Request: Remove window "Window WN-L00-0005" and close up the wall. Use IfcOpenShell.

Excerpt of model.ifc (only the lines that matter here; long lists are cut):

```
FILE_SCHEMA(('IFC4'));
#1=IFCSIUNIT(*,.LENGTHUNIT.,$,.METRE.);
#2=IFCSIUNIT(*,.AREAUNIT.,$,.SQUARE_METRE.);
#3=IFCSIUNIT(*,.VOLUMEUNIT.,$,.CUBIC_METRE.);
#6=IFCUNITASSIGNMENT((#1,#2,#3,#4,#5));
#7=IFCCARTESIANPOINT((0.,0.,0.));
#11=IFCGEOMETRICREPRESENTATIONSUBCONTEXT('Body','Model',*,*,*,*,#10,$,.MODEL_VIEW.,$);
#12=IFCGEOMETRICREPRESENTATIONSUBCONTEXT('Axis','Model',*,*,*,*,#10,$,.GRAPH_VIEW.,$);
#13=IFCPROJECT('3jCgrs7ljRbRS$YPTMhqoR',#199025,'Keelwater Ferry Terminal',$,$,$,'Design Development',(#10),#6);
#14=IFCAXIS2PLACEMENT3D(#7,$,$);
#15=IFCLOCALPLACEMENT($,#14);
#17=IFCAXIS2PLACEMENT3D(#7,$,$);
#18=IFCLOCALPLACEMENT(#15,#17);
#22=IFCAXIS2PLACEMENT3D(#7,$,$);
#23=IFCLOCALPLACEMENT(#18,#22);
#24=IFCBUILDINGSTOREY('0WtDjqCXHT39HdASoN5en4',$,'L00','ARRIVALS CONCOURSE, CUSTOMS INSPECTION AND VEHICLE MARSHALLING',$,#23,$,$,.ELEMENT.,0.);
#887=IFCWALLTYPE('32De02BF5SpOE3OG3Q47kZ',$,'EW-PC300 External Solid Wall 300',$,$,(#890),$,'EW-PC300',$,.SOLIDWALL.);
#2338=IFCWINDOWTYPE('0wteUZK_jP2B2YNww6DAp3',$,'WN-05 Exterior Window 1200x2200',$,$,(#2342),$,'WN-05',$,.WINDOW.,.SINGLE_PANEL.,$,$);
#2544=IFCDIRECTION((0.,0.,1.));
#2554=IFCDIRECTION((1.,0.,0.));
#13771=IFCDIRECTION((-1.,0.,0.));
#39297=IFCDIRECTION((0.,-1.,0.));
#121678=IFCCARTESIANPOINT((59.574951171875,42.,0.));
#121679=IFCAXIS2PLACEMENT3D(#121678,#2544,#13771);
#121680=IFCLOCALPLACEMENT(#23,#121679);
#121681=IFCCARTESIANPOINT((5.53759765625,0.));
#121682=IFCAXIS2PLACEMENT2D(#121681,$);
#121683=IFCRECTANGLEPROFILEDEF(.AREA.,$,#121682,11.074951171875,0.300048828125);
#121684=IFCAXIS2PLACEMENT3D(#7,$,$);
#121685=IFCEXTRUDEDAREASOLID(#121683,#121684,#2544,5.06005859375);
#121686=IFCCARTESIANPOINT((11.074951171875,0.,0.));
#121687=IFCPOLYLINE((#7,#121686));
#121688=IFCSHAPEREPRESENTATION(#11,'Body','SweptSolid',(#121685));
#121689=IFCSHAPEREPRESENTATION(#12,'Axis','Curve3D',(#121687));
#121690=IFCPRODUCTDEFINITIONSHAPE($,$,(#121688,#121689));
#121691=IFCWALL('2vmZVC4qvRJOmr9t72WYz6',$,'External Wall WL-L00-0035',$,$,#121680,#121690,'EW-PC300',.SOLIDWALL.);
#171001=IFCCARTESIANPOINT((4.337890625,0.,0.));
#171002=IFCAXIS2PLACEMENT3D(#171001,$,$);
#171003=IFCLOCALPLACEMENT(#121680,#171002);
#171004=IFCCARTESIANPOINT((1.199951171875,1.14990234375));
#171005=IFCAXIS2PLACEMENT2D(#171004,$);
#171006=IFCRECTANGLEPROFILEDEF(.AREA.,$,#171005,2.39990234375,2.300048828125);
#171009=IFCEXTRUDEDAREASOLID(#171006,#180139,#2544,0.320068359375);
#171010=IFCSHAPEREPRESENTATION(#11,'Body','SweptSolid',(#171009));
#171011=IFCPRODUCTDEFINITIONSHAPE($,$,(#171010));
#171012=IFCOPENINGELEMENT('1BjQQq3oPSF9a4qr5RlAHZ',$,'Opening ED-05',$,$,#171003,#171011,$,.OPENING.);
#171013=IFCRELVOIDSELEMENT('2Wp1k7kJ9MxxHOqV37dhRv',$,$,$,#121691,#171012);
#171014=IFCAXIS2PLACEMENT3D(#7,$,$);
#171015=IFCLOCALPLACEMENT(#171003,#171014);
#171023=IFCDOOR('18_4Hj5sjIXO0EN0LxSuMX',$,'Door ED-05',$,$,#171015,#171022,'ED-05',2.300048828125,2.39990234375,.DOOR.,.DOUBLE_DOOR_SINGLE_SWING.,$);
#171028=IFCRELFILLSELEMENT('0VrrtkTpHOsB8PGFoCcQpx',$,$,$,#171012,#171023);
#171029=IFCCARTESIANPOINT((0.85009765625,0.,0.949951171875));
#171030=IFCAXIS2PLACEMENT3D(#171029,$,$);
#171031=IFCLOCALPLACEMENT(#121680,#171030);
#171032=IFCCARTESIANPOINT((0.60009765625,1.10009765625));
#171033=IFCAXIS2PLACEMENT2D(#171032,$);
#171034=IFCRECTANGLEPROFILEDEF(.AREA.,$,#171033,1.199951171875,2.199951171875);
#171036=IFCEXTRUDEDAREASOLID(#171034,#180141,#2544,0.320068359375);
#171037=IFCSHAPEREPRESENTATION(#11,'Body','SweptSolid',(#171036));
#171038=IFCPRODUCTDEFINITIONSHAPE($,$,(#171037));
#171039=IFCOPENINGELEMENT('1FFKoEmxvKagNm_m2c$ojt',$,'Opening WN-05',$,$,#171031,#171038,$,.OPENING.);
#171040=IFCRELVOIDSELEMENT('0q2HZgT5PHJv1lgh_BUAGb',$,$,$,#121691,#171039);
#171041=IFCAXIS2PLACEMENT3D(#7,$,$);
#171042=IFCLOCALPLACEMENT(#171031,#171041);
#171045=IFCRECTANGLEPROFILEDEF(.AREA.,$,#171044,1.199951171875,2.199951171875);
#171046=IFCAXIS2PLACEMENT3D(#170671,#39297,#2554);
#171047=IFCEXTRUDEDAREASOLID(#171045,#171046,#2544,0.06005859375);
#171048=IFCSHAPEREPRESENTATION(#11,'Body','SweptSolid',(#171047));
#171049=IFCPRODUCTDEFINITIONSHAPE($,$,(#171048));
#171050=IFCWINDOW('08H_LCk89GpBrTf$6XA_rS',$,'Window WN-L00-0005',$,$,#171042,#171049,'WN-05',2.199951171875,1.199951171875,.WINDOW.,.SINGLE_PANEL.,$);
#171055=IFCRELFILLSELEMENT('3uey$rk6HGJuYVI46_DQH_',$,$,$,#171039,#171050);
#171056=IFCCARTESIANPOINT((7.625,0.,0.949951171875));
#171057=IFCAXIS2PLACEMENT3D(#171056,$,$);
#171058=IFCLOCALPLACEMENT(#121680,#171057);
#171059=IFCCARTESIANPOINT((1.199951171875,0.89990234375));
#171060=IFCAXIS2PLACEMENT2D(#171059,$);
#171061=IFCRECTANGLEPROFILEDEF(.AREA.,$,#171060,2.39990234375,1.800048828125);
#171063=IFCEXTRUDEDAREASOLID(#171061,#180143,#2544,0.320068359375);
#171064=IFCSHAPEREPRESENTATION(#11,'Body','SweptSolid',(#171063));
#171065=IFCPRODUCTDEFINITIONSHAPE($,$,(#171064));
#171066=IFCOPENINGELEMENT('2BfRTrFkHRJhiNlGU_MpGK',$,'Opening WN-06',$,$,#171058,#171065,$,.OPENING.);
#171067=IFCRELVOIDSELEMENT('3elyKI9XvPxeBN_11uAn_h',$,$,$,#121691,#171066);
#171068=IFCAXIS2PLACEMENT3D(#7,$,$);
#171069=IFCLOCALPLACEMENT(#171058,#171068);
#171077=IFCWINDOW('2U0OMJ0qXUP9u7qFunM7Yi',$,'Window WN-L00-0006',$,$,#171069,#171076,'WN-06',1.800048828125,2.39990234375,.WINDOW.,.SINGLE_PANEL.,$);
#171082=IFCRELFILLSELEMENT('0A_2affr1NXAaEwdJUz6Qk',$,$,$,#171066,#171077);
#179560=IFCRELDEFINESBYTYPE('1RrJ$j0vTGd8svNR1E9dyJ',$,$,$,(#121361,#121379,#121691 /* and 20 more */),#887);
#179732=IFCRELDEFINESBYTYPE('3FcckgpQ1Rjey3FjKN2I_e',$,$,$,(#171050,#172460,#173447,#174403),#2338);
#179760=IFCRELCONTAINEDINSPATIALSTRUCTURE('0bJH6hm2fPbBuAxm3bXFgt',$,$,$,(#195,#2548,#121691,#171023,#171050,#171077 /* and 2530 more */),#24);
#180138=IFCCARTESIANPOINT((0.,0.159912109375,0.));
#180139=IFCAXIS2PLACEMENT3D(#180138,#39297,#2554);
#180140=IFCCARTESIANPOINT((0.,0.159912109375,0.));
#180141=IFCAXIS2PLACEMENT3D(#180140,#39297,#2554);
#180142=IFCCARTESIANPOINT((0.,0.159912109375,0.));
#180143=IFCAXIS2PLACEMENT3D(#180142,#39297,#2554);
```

```python
import ifcopenshell
import ifcopenshell.api.feature
import ifcopenshell.api.root
import ifcopenshell.geom
import ifcopenshell.util.shape

model = ifcopenshell.open("model.ifc")
settings = ifcopenshell.geom.settings()


def volume(element):
    """Net volume in cubic metres, openings subtracted."""
    shape = ifcopenshell.geom.create_shape(settings, element)
    return ifcopenshell.util.shape.get_volume(shape.geometry)


window = model.by_guid("08H_LCk89GpBrTf$6XA_rS")
opening = window.FillsVoids[0].RelatingOpeningElement
wall = opening.VoidsElements[0].RelatingBuildingElement
before = volume(wall)

ifcopenshell.api.root.remove_product(model, product=window)
ifcopenshell.api.feature.remove_feature(model, feature=opening)

after = volume(wall)

print(f"wall volume {before:.3f} -> {after:.3f} m3")

model.write("model_edited.ifc")
```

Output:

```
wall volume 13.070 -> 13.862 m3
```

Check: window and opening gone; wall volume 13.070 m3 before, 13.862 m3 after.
